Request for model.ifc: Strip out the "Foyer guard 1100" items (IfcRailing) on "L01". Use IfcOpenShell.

First a look at what the model holds.

```python
import ifcopenshell
import ifcopenshell.util.element

model = ifcopenshell.open("model.ifc")
print(model.schema)
storey = next(s for s in model.by_type("IfcBuildingStorey") if s.Name == "L01")
railings = [e for e in ifcopenshell.util.element.get_decomposition(storey) if e.is_a("IfcRailing")]
seen = {}
for e in railings:
    element_type = ifcopenshell.util.element.get_type(e)
    name = element_type.Name if element_type not in (None, e) else None
    seen[name] = seen.get(name, 0) + 1
for name, count in sorted(seen.items(), key=str):
    print(count, "x", name)
```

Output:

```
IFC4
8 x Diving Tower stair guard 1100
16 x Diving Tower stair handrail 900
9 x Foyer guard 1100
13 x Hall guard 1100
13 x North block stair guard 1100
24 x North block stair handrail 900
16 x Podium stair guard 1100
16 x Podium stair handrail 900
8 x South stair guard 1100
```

```python
import ifcopenshell
import ifcopenshell.api.root
import ifcopenshell.util.element

model = ifcopenshell.open("model.ifc")

storey = next(s for s in model.by_type("IfcBuildingStorey") if s.Name == "L01")
railings = [e for e in ifcopenshell.util.element.get_decomposition(storey) if e.is_a("IfcRailing")]
targets = [e for e in railings if (t := ifcopenshell.util.element.get_type(e)) not in (None, e) and t.Name == "Foyer guard 1100"]

for e in targets:
    ifcopenshell.api.root.remove_product(model, product=e)
print(len(targets), "removed")

model.write("model_updated.ifc")
```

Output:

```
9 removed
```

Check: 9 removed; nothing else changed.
